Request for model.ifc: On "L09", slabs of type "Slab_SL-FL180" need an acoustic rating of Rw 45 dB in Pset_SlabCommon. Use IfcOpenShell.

First a look at what the model holds.

```python
import ifcopenshell
import ifcopenshell.util.element

model = ifcopenshell.open("model.ifc")
print(model.schema)
storey = next(s for s in model.by_type("IfcBuildingStorey") if s.Name == "L09")
slabs = [e for e in ifcopenshell.util.element.get_decomposition(storey) if e.is_a("IfcSlab")]
seen = {}
for e in slabs:
    element_type = ifcopenshell.util.element.get_type(e)
    key = (element_type.Name if element_type != e and element_type else None, ifcopenshell.util.element.get_pset(e, "Pset_SlabCommon", "AcousticRating"))
    seen[key] = seen.get(key, 0) + 1
for (name, value), count in sorted(seen.items(), key=str):
    print(count, "x", name, "|", value)
```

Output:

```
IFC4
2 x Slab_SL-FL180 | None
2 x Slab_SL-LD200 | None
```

```python
import ifcopenshell
import ifcopenshell.api.pset
import ifcopenshell.util.element

model = ifcopenshell.open("model.ifc")

storey = next(s for s in model.by_type("IfcBuildingStorey") if s.Name == "L09")
slabs = [e for e in ifcopenshell.util.element.get_decomposition(storey) if e.is_a("IfcSlab")]

count = 0
for e in slabs:
    element_type = ifcopenshell.util.element.get_type(e)
    if element_type in (None, e) or element_type.Name != "Slab_SL-FL180":
        continue
    # add_pset returns the element's existing set when there is one.
    pset = ifcopenshell.api.pset.add_pset(model, product=e, name="Pset_SlabCommon")
    ifcopenshell.api.pset.edit_pset(model, pset=pset, properties={"AcousticRating": "Rw 45 dB"})
    count += 1

print(count, "slabs updated")

model.write("model_updated.ifc")
```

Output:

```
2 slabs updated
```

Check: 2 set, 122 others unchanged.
